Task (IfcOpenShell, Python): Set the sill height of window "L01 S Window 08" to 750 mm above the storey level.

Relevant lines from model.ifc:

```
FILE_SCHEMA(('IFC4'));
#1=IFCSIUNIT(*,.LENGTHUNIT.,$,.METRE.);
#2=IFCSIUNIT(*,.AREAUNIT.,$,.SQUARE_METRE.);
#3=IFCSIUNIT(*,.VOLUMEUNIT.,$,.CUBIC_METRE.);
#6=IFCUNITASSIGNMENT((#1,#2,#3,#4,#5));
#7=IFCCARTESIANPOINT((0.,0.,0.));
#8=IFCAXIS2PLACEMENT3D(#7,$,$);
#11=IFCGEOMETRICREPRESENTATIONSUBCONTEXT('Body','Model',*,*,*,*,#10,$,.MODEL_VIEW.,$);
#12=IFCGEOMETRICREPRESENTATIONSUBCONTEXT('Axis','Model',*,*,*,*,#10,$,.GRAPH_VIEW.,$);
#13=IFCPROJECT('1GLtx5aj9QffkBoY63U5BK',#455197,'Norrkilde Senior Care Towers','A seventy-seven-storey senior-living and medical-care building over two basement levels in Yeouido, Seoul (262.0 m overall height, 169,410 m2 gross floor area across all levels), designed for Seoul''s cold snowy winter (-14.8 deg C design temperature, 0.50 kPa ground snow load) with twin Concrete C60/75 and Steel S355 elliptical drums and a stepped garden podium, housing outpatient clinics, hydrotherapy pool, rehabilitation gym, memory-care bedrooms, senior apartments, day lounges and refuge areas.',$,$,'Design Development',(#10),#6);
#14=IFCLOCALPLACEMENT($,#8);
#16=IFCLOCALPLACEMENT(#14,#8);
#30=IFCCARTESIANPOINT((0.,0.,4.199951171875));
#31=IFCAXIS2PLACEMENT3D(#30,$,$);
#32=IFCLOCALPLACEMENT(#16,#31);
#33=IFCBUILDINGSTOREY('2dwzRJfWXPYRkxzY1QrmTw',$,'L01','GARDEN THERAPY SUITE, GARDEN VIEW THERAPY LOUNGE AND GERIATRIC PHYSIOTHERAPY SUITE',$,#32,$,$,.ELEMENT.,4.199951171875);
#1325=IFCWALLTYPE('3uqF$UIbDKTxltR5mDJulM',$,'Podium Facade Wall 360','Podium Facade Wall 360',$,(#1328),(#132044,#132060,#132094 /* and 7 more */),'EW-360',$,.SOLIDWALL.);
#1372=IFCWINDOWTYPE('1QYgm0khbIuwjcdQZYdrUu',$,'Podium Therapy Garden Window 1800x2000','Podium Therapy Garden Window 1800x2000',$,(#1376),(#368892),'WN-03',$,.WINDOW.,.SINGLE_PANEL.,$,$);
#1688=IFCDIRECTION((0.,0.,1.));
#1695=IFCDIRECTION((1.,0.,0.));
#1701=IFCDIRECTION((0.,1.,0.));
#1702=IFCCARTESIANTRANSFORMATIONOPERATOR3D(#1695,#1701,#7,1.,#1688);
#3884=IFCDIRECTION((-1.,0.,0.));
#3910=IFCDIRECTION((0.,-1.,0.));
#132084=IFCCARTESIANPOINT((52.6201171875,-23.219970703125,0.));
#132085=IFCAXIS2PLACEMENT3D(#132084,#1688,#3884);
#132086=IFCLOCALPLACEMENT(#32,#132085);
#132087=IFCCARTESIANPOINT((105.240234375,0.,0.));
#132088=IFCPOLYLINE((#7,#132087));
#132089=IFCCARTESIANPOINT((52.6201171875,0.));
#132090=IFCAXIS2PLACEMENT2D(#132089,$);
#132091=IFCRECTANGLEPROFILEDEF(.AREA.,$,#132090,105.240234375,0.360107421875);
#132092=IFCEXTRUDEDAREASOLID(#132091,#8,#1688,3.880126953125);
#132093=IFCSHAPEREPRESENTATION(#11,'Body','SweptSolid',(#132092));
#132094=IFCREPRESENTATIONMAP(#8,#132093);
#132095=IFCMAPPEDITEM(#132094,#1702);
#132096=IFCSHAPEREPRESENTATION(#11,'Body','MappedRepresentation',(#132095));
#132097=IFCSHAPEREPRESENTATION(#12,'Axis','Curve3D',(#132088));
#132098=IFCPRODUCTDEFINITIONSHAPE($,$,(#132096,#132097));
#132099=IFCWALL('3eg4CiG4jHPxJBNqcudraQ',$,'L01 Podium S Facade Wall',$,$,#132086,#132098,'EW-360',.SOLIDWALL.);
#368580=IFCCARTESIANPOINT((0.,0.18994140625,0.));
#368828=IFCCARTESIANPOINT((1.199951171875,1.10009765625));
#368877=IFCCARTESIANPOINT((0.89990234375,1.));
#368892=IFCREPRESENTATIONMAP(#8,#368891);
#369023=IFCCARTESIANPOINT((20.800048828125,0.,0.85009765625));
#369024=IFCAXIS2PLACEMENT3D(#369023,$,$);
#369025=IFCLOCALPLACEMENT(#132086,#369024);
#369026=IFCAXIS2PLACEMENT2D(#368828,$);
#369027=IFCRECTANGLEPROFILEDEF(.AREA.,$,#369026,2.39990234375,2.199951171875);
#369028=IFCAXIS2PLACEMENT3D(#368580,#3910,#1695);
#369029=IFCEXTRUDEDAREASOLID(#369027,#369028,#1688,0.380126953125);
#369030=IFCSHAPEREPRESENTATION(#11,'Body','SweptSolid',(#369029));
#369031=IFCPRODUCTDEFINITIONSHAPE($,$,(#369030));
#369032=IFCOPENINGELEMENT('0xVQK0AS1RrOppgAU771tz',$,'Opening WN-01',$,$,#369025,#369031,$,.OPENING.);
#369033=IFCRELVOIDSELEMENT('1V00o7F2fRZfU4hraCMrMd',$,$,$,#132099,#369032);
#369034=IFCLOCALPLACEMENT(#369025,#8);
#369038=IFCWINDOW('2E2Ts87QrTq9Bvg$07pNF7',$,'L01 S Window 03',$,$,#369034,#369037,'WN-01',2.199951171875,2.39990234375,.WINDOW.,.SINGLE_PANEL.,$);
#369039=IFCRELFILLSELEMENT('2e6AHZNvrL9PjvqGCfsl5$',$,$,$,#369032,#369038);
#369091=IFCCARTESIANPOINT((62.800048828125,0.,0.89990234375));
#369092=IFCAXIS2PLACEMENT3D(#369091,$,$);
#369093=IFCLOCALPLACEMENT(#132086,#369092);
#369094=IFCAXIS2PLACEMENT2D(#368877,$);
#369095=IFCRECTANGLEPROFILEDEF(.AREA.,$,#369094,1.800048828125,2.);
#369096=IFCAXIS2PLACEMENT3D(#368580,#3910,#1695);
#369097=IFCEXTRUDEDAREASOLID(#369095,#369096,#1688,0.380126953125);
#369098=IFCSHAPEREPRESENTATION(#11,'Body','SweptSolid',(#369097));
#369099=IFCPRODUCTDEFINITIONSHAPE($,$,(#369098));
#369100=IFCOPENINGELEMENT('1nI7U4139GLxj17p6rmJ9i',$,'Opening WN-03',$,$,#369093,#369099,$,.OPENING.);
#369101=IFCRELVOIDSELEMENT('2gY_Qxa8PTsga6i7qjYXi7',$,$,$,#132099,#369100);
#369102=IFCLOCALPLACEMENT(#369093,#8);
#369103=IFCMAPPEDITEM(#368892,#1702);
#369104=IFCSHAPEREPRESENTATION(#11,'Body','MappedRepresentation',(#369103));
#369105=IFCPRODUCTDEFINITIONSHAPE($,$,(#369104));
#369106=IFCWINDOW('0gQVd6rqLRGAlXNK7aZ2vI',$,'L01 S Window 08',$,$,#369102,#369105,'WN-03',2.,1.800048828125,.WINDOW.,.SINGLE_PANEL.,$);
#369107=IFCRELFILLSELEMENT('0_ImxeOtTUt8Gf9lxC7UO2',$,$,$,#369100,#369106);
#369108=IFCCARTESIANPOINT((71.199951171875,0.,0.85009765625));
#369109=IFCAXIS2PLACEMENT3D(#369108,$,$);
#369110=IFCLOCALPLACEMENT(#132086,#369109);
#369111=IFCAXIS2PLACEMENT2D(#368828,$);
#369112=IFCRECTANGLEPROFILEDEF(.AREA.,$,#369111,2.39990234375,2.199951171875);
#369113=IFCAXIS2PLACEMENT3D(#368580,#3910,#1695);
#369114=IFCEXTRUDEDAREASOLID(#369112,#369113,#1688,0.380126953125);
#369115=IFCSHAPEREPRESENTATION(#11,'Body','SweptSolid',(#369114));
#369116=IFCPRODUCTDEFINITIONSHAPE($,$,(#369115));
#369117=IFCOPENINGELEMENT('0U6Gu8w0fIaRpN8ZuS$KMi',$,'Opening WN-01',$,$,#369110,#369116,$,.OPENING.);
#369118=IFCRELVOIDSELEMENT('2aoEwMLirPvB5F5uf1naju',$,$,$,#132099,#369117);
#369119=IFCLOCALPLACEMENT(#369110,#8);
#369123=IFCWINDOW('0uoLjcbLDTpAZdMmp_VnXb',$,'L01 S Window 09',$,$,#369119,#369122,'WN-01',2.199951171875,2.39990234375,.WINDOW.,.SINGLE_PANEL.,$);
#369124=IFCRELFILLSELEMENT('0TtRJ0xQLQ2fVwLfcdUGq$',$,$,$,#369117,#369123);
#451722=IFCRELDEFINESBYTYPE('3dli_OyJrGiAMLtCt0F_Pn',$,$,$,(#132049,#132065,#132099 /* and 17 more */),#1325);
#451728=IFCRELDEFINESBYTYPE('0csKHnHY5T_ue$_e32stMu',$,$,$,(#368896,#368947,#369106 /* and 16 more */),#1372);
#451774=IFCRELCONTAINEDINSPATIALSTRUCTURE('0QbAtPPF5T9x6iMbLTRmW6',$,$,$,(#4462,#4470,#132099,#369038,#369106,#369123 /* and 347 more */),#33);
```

```python
import numpy as np
import ifcopenshell
import ifcopenshell.api.geometry
import ifcopenshell.geom
import ifcopenshell.util.element
import ifcopenshell.util.placement
import ifcopenshell.util.shape
import ifcopenshell.util.unit

model = ifcopenshell.open("model.ifc")
unit_scale = ifcopenshell.util.unit.calculate_unit_scale(model)

window = model.by_id(369106)
opening = window.FillsVoids[0].RelatingOpeningElement
storey = ifcopenshell.util.element.get_container(window, ifc_class="IfcBuildingStorey")
level = ifcopenshell.util.placement.get_local_placement(storey.ObjectPlacement)[2, 3]

# The opening's origin need not be at the sill, so measure its lowest point.
shape = ifcopenshell.geom.create_shape(ifcopenshell.geom.settings(), opening)
bottom = ifcopenshell.util.shape.get_shape_bottom_elevation(shape, shape.geometry) / unit_scale
dz = level + 0.75 - bottom

shift = np.array([0.0, 0.0, dz])
# The window is placed relative to its opening, so it follows when the opening moves.
matrix = ifcopenshell.util.placement.get_local_placement(opening.ObjectPlacement)
matrix[:3, 3] += shift
ifcopenshell.api.geometry.edit_object_placement(
    model, product=opening, matrix=matrix, is_si=False, should_transform_children=True
)

print(f"moved by {dz * unit_scale:+.3f} m")

model.write("model_rev.ifc")
```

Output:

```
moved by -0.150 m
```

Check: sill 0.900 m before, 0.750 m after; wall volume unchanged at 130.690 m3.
